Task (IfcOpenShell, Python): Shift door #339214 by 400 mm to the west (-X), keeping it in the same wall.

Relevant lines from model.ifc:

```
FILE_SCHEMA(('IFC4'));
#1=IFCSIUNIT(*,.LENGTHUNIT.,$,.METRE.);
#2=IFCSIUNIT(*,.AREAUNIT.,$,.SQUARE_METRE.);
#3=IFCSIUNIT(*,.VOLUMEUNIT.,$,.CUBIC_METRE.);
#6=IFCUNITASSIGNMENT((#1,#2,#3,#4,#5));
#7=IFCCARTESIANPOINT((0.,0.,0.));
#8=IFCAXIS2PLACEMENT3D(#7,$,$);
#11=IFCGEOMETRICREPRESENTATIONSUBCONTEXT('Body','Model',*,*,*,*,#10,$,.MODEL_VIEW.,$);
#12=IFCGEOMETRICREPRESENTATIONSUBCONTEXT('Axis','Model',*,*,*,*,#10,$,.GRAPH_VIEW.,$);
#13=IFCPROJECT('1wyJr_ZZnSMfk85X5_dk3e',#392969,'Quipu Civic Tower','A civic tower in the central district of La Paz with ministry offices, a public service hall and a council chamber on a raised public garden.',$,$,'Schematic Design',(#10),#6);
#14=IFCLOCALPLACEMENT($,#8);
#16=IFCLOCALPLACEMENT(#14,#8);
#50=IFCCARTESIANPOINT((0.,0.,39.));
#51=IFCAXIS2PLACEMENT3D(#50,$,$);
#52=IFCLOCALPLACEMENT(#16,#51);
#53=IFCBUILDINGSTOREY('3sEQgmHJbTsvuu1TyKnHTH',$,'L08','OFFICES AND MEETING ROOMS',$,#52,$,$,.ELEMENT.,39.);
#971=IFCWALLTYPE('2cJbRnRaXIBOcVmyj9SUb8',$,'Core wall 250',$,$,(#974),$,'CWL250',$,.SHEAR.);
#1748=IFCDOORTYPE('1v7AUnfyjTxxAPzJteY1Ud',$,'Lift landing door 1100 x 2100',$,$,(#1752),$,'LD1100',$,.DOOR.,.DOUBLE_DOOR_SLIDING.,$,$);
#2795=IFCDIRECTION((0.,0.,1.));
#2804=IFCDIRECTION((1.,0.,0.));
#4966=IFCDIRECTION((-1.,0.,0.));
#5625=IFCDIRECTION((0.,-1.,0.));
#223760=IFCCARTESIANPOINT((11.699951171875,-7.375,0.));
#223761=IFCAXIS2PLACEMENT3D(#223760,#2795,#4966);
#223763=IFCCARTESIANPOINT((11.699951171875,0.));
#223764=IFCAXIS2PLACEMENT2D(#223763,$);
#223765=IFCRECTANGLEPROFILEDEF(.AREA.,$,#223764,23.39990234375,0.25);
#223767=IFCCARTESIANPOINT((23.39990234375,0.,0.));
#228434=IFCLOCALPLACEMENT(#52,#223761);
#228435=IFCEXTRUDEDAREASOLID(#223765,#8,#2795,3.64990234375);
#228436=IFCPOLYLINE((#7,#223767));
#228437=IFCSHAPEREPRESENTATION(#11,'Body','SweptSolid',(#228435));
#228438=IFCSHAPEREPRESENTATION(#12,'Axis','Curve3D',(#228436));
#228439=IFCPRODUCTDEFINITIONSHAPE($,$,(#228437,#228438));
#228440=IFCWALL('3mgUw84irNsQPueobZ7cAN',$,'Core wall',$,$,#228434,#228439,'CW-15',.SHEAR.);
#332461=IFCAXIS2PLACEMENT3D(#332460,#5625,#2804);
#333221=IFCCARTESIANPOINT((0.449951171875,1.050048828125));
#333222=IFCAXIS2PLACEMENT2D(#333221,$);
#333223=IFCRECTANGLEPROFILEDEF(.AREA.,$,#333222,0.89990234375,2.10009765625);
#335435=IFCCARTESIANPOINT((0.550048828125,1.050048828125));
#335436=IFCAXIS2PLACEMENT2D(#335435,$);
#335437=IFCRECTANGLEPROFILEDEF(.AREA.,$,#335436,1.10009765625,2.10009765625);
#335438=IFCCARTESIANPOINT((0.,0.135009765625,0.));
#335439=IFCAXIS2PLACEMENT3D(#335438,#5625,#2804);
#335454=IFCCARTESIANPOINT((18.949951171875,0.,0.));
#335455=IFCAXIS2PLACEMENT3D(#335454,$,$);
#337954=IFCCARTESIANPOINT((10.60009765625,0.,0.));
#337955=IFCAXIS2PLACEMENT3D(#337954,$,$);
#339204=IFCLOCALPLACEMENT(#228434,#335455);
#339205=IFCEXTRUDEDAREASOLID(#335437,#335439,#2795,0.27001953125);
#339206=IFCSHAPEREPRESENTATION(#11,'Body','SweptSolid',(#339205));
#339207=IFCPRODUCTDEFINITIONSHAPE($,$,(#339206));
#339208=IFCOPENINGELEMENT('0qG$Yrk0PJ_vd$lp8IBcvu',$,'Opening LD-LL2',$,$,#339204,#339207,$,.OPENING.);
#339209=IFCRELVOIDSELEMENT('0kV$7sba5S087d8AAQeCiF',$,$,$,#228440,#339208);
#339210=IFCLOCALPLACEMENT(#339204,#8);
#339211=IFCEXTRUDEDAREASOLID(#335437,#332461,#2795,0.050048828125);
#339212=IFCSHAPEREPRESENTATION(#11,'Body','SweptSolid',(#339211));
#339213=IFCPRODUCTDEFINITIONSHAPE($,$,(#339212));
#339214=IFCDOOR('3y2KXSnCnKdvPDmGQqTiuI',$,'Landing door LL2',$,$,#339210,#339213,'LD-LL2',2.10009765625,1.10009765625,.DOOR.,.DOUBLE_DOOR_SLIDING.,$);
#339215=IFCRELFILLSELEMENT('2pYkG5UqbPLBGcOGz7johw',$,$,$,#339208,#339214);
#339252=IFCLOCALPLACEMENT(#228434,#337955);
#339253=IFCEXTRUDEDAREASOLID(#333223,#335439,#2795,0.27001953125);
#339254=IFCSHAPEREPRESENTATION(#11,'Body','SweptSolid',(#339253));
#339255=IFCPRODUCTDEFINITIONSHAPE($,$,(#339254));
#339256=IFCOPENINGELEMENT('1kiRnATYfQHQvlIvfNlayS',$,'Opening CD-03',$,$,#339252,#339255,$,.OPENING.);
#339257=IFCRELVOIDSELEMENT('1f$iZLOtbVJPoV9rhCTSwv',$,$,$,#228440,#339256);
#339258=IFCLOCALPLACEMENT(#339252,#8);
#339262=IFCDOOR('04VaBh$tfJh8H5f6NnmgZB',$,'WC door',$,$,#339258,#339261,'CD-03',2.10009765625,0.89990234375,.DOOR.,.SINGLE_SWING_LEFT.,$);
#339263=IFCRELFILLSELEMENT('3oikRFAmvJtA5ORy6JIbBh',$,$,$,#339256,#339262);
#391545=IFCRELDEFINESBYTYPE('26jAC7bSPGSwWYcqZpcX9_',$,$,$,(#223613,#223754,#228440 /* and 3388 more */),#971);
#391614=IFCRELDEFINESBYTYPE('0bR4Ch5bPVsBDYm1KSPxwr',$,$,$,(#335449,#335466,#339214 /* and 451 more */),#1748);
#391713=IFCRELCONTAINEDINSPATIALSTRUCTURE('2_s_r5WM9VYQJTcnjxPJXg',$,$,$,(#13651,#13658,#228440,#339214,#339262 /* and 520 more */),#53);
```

```python
import ifcopenshell
import ifcopenshell.api.geometry
import ifcopenshell.util.placement
import ifcopenshell.util.unit

model = ifcopenshell.open("model.ifc")
unit_scale = ifcopenshell.util.unit.calculate_unit_scale(model)

door = model.by_guid("3y2KXSnCnKdvPDmGQqTiuI")
opening = door.FillsVoids[0].RelatingOpeningElement
wall = opening.VoidsElements[0].RelatingBuildingElement

wall_matrix = ifcopenshell.util.placement.get_local_placement(wall.ObjectPlacement)
shift = wall_matrix[:3, 0] * 0.4 / unit_scale
before = ifcopenshell.util.placement.get_local_placement(door.ObjectPlacement)[:3, 3].copy()

# The door is placed relative to its opening, so it follows when the opening moves.
matrix = ifcopenshell.util.placement.get_local_placement(opening.ObjectPlacement)
matrix[:3, 3] += shift
ifcopenshell.api.geometry.edit_object_placement(
    model, product=opening, matrix=matrix, is_si=False, should_transform_children=True
)

after = ifcopenshell.util.placement.get_local_placement(door.ObjectPlacement)[:3, 3]
print("door moved by", (after - before).round(3) + 0.0)

model.write("model_rev.ifc")
```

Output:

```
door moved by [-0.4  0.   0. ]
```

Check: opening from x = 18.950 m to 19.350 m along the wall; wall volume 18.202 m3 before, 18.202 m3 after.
